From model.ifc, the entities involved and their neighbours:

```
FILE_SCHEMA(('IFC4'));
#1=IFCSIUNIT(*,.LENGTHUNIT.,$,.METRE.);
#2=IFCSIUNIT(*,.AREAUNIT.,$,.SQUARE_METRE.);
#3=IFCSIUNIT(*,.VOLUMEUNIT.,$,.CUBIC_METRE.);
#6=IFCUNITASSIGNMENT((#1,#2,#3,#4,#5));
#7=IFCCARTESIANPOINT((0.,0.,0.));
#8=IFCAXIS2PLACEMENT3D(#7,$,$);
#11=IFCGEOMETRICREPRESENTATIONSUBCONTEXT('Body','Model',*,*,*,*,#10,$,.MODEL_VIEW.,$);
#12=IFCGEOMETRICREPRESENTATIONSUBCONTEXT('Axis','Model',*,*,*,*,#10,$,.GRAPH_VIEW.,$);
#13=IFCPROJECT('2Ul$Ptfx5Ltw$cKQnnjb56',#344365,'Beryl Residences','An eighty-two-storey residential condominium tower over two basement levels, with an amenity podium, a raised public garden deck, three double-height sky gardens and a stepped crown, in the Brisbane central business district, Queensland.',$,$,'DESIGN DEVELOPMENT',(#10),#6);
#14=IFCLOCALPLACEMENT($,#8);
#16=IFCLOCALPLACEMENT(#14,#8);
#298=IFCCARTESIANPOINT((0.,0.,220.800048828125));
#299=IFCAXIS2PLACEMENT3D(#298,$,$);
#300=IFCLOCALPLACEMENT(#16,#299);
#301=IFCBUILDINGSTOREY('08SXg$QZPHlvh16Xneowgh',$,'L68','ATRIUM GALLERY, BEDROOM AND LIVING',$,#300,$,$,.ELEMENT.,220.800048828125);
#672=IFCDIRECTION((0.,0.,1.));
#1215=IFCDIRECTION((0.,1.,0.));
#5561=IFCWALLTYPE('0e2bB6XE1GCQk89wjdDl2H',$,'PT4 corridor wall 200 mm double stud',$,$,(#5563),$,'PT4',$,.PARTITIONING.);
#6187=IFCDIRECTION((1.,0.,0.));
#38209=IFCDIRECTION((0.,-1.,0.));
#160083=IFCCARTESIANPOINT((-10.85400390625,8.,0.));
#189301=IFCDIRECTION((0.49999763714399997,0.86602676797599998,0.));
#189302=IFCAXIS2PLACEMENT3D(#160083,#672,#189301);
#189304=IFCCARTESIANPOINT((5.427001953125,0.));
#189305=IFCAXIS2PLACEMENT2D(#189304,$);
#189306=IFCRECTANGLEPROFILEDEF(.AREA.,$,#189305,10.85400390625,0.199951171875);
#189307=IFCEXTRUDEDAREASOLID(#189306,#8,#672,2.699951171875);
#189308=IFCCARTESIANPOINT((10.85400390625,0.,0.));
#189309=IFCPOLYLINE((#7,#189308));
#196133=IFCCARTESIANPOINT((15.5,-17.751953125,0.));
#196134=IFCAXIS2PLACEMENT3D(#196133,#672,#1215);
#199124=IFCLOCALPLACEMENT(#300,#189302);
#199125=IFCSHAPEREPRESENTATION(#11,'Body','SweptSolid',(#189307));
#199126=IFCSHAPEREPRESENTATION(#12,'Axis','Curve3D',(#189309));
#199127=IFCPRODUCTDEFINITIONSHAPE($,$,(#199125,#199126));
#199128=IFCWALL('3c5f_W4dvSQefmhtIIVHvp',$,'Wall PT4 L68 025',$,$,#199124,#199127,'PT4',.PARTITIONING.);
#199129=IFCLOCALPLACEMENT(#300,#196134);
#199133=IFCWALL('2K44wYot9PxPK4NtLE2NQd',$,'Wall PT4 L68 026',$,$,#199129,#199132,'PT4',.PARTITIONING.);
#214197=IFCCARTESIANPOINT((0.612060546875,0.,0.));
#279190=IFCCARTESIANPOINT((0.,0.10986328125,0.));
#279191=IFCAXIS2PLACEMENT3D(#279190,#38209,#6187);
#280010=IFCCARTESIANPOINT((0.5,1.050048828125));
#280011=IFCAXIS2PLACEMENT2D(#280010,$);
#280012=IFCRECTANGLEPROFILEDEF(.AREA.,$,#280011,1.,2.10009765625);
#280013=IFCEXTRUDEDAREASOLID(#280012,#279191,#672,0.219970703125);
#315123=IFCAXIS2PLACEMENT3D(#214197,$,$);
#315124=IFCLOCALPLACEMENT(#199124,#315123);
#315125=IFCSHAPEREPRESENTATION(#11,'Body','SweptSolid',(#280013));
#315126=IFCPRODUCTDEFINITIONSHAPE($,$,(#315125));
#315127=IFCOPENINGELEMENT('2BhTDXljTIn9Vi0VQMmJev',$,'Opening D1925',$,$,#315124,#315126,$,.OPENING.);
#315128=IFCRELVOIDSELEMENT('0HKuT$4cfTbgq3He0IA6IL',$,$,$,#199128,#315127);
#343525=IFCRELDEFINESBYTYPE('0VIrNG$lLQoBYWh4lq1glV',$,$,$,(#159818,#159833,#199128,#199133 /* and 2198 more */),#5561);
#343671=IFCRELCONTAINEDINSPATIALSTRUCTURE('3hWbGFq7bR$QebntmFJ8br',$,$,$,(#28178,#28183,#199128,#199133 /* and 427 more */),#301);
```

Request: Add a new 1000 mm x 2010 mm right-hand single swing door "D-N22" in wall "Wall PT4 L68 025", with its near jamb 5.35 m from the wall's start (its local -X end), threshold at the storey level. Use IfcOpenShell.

```python
import numpy as np
import ifcopenshell
import ifcopenshell.api.feature
import ifcopenshell.api.geometry
import ifcopenshell.api.root
import ifcopenshell.api.spatial
import ifcopenshell.geom
import ifcopenshell.util.element
import ifcopenshell.util.placement
import ifcopenshell.util.representation
import ifcopenshell.util.shape
import ifcopenshell.util.unit

model = ifcopenshell.open("model.ifc")
unit_scale = ifcopenshell.util.unit.calculate_unit_scale(model)
settings = ifcopenshell.geom.settings()


def volume(element):
    """Net volume in cubic metres, openings subtracted."""
    shape = ifcopenshell.geom.create_shape(settings, element)
    return ifcopenshell.util.shape.get_volume(shape.geometry)


wall = model.by_guid("3c5f_W4dvSQefmhtIIVHvp")
storey = ifcopenshell.util.element.get_container(wall, ifc_class="IfcBuildingStorey")
context = ifcopenshell.util.representation.get_context(model, "Model", "Body", "MODEL_VIEW")
before = volume(wall)

width, height, from_end, sill = 1, 2.01, 5.35, 0.0  # metres

# The wall runs along its own X axis, and the end named is its -X end.
wall_shape = ifcopenshell.geom.create_shape(settings, wall)
x, y, z = ifcopenshell.util.shape.get_vertices(wall_shape.geometry).T
start = x.min() + from_end
face, thickness = float(y.min()), float(y.max() - y.min())
wall_matrix = ifcopenshell.util.placement.get_local_placement(wall.ObjectPlacement)
level = ifcopenshell.util.placement.get_local_placement(storey.ObjectPlacement)[2, 3]


def in_wall(x, y):
    """Placement at x, y metres in the wall's axes, at sill height."""
    matrix = wall_matrix.copy()
    matrix[:, 3] = wall_matrix @ np.array([x / unit_scale, y / unit_scale, 0.0, 1.0])
    matrix[2, 3] = level + sill / unit_scale
    return matrix


# Opening: a box that overshoots both wall faces by 50 mm.
opening = ifcopenshell.api.root.create_entity(model, ifc_class="IfcOpeningElement", predefined_type="OPENING")
box = ifcopenshell.api.geometry.add_wall_representation(
    model, context=context, length=width, height=height, thickness=thickness + 0.1
)
ifcopenshell.api.geometry.assign_representation(model, product=opening, representation=box)
ifcopenshell.api.geometry.edit_object_placement(model, product=opening, matrix=in_wall(start, face - 0.05), is_si=False)
ifcopenshell.api.feature.add_feature(model, feature=opening, element=wall)

door = ifcopenshell.api.root.create_entity(model, ifc_class="IfcDoor", name="D-N22", predefined_type="DOOR")
door.OverallWidth, door.OverallHeight = width / unit_scale, height / unit_scale
door.OperationType = "SINGLE_SWING_RIGHT"
body = ifcopenshell.api.geometry.add_door_representation(
    model,
    context=context,
    overall_width=door.OverallWidth,
    overall_height=door.OverallHeight,
    operation_type="SINGLE_SWING_RIGHT",
    lining_properties={"LiningDepth": thickness / unit_scale, "ThresholdDepth": thickness / unit_scale},
)
ifcopenshell.api.geometry.assign_representation(model, product=door, representation=body)
ifcopenshell.api.spatial.assign_container(model, products=[door], relating_structure=storey)
ifcopenshell.api.feature.add_filling(model, opening=opening, element=door)

# The lining spans the wall, so the door starts at the wall face.
ifcopenshell.api.geometry.edit_object_placement(model, product=door, matrix=in_wall(start, face), is_si=False)

after = volume(wall)

print(f"wall volume {before:.3f} -> {after:.3f} m3")

model.write("model_rev.ifc")
```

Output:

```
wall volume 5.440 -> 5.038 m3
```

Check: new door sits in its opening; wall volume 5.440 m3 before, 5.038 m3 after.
